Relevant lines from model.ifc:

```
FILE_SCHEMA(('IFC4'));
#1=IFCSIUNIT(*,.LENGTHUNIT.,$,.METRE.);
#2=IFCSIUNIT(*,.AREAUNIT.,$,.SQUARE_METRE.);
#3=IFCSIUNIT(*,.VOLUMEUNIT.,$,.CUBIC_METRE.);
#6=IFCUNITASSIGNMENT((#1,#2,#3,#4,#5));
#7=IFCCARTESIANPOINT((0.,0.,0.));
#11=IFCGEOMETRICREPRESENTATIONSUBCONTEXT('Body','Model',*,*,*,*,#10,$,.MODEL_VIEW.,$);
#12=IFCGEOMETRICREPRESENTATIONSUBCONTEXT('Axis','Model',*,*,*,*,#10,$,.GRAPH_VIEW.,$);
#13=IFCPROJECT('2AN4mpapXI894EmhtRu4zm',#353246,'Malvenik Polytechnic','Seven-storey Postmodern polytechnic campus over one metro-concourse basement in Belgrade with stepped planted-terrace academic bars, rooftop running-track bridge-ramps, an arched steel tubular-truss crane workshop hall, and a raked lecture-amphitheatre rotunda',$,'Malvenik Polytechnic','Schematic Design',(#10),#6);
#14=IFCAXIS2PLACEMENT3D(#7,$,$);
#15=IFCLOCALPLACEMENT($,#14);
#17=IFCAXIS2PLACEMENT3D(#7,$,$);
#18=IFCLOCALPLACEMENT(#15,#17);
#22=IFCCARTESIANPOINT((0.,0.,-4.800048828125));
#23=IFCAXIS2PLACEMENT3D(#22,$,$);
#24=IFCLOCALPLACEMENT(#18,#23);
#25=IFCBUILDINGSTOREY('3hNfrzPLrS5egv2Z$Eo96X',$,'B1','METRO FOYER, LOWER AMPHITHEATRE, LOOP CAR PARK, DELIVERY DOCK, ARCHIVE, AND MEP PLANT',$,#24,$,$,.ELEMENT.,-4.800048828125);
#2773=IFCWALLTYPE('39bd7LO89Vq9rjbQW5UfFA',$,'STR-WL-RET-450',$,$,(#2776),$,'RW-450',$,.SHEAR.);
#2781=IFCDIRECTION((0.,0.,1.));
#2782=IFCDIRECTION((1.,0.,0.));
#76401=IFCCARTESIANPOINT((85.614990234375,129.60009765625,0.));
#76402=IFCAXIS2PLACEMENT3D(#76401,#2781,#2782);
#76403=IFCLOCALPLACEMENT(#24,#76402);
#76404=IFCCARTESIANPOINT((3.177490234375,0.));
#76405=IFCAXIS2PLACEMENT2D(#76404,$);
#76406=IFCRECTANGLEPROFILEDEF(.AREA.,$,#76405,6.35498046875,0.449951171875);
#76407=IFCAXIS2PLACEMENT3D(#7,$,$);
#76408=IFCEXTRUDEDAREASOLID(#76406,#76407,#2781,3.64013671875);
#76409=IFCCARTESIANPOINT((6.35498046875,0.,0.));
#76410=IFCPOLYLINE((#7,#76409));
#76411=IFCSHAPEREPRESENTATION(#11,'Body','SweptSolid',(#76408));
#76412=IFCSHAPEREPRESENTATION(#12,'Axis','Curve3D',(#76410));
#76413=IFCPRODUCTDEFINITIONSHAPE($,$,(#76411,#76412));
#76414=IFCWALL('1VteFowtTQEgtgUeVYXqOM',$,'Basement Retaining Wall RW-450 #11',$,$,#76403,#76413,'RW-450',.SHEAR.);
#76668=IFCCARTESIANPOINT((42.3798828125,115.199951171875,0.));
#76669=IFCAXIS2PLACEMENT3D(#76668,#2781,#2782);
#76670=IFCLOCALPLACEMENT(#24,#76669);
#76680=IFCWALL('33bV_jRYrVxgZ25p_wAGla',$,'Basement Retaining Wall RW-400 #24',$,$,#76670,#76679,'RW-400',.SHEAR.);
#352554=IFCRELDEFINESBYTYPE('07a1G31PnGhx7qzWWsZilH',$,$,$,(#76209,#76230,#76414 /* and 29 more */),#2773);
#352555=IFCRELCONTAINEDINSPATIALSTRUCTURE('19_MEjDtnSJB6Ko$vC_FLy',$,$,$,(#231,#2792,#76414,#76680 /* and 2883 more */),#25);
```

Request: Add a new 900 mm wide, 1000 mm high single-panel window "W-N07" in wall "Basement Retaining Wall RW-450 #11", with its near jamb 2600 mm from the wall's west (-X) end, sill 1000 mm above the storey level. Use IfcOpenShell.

```python
import numpy as np
import ifcopenshell
import ifcopenshell.api.feature
import ifcopenshell.api.geometry
import ifcopenshell.api.root
import ifcopenshell.api.spatial
import ifcopenshell.geom
import ifcopenshell.util.element
import ifcopenshell.util.placement
import ifcopenshell.util.representation
import ifcopenshell.util.shape
import ifcopenshell.util.unit

model = ifcopenshell.open("model.ifc")
unit_scale = ifcopenshell.util.unit.calculate_unit_scale(model)
settings = ifcopenshell.geom.settings()


def volume(element):
    """Net volume in cubic metres, openings subtracted."""
    shape = ifcopenshell.geom.create_shape(settings, element)
    return ifcopenshell.util.shape.get_volume(shape.geometry)


wall = model.by_guid("1VteFowtTQEgtgUeVYXqOM")
storey = ifcopenshell.util.element.get_container(wall, ifc_class="IfcBuildingStorey")
context = ifcopenshell.util.representation.get_context(model, "Model", "Body", "MODEL_VIEW")
before = volume(wall)

width, height, from_end, sill = 0.9, 1, 2.6, 1  # metres

# The wall runs along its own X axis, and the end named is its -X end.
wall_shape = ifcopenshell.geom.create_shape(settings, wall)
x, y, z = ifcopenshell.util.shape.get_vertices(wall_shape.geometry).T
start = x.min() + from_end
face, thickness = float(y.min()), float(y.max() - y.min())
wall_matrix = ifcopenshell.util.placement.get_local_placement(wall.ObjectPlacement)
level = ifcopenshell.util.placement.get_local_placement(storey.ObjectPlacement)[2, 3]


def in_wall(x, y):
    """Placement at x, y metres in the wall's axes, at sill height."""
    matrix = wall_matrix.copy()
    matrix[:, 3] = wall_matrix @ np.array([x / unit_scale, y / unit_scale, 0.0, 1.0])
    matrix[2, 3] = level + sill / unit_scale
    return matrix


# Opening: a box that overshoots both wall faces by 50 mm.
opening = ifcopenshell.api.root.create_entity(model, ifc_class="IfcOpeningElement", predefined_type="OPENING")
box = ifcopenshell.api.geometry.add_wall_representation(
    model, context=context, length=width, height=height, thickness=thickness + 0.1
)
ifcopenshell.api.geometry.assign_representation(model, product=opening, representation=box)
ifcopenshell.api.geometry.edit_object_placement(model, product=opening, matrix=in_wall(start, face - 0.05), is_si=False)
ifcopenshell.api.feature.add_feature(model, feature=opening, element=wall)

window = ifcopenshell.api.root.create_entity(model, ifc_class="IfcWindow", name="W-N07", predefined_type="WINDOW")
window.OverallWidth, window.OverallHeight = width / unit_scale, height / unit_scale
window.PartitioningType = "SINGLE_PANEL"
body = ifcopenshell.api.geometry.add_window_representation(
    model,
    context=context,
    overall_width=window.OverallWidth,
    overall_height=window.OverallHeight,
    partition_type="SINGLE_PANEL",
)
ifcopenshell.api.geometry.assign_representation(model, product=window, representation=body)
ifcopenshell.api.spatial.assign_container(model, products=[window], relating_structure=storey)
ifcopenshell.api.feature.add_filling(model, opening=opening, element=window)

# Centre the window in the wall's thickness.
ifcopenshell.api.geometry.edit_object_placement(model, product=window, matrix=in_wall(start, face), is_si=False)
window_shape = ifcopenshell.geom.create_shape(settings, window)
depth = ifcopenshell.util.shape.get_vertices(window_shape.geometry)[:, 1]
offset = face + thickness / 2 - (depth.min() + depth.max()) / 2
ifcopenshell.api.geometry.edit_object_placement(model, product=window, matrix=in_wall(start, offset), is_si=False)

after = volume(wall)

print(f"wall volume {before:.3f} -> {after:.3f} m3")

model.write("model_v2.ifc")
```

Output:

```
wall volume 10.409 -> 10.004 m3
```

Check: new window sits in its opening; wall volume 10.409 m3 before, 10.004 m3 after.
